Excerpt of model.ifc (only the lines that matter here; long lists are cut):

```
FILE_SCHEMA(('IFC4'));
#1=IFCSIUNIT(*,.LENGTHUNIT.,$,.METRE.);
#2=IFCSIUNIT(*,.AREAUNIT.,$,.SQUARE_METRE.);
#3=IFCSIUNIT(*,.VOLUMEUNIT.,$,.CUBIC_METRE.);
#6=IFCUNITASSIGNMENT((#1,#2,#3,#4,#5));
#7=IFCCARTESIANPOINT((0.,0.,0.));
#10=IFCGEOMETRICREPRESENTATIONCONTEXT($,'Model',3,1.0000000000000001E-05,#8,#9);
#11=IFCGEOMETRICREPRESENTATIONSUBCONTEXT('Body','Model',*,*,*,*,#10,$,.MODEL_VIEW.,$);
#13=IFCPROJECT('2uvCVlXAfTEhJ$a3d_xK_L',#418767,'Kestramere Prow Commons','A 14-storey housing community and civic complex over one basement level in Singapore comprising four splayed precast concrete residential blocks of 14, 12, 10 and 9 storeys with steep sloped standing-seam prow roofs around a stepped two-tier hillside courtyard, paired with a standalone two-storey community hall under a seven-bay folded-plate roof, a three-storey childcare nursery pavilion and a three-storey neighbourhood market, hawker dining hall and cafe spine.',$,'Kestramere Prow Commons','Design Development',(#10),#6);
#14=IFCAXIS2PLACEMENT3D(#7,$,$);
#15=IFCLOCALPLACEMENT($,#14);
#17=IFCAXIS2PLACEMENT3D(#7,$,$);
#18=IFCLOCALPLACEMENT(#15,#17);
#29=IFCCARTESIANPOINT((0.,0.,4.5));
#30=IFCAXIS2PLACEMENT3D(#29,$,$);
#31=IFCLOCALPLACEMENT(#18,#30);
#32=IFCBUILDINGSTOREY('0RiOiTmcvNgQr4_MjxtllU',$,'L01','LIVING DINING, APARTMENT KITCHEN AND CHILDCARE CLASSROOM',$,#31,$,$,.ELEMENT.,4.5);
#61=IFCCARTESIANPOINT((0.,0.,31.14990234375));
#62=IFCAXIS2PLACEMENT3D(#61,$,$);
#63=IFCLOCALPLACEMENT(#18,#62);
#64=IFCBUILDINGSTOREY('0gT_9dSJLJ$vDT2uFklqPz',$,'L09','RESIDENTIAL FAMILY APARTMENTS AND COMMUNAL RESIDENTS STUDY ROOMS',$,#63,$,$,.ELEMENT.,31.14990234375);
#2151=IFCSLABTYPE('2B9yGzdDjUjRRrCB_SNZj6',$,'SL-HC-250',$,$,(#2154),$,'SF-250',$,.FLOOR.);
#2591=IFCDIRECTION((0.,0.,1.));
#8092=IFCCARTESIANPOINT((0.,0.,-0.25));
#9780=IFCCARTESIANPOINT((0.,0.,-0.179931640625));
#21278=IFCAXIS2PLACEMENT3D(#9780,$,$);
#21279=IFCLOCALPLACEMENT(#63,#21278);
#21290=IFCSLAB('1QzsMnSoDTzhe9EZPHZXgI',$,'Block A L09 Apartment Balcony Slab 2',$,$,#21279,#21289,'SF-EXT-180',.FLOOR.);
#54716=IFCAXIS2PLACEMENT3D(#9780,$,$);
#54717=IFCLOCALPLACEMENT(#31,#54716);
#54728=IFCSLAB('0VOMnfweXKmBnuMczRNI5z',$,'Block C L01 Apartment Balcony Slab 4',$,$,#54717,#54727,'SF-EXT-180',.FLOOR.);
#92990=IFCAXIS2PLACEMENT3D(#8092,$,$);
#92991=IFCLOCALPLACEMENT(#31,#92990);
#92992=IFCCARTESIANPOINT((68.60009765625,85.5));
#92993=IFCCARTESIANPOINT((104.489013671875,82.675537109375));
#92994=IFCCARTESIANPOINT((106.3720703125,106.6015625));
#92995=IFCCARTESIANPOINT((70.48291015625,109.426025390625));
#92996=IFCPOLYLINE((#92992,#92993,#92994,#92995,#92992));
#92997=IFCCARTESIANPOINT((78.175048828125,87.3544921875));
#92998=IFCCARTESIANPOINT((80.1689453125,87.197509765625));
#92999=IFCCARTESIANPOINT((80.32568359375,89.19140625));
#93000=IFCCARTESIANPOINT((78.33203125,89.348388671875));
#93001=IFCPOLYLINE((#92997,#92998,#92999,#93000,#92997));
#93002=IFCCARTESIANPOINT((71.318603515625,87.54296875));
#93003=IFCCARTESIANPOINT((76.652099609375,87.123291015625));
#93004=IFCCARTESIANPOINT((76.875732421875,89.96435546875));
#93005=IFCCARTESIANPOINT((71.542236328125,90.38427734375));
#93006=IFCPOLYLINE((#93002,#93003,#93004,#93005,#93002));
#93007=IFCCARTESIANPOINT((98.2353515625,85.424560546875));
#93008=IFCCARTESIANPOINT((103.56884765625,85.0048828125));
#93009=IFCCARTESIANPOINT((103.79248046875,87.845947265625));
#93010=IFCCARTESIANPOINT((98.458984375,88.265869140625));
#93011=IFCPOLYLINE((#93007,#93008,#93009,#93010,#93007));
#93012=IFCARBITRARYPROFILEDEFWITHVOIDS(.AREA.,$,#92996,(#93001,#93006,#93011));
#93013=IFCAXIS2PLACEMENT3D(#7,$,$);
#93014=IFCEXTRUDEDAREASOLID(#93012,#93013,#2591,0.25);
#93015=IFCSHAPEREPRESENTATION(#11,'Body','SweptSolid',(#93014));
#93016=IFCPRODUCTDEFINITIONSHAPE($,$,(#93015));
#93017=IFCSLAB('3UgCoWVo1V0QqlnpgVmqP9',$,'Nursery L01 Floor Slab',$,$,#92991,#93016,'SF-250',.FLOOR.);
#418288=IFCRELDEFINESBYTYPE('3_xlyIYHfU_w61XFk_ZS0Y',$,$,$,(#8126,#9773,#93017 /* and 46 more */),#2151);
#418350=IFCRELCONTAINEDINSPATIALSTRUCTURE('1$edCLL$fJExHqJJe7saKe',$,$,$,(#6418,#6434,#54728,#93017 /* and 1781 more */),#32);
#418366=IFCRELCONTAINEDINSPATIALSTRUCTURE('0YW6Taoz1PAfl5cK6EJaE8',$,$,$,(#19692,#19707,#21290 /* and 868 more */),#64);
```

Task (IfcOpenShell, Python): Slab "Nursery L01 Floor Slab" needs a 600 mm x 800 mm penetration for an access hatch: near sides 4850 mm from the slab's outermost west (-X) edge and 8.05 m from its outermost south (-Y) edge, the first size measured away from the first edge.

```python
import numpy as np
import ifcopenshell
import ifcopenshell.api.feature
import ifcopenshell.api.geometry
import ifcopenshell.api.root
import ifcopenshell.geom
import ifcopenshell.util.placement
import ifcopenshell.util.representation
import ifcopenshell.util.shape
import ifcopenshell.util.unit

model = ifcopenshell.open("model.ifc")
unit_scale = ifcopenshell.util.unit.calculate_unit_scale(model)
settings = ifcopenshell.geom.settings()


def volume(element):
    """Net volume in cubic metres, openings subtracted."""
    shape = ifcopenshell.geom.create_shape(settings, element)
    return ifcopenshell.util.shape.get_volume(shape.geometry)


slab = model.by_guid("3UgCoWVo1V0QqlnpgVmqP9")
before = volume(slab)

# Extent in the slab's own axes, in metres. The edges named are its -X and -Y sides.
slab_shape = ifcopenshell.geom.create_shape(settings, slab)
vertices = ifcopenshell.util.shape.get_vertices(slab_shape.geometry)
x_min, y_min, bottom = vertices.min(axis=0)
top = vertices[:, 2].max()

opening = ifcopenshell.api.root.create_entity(model, ifc_class="IfcOpeningElement", name="Access hatch opening", predefined_type="OPENING")
context = ifcopenshell.util.representation.get_context(model, "Model", "Body", "MODEL_VIEW")
width, depth = 0.6, 0.8
outline = [(0.0, 0.0), (width, 0.0), (width, depth), (0.0, depth), (0.0, 0.0)]
# Overshoot both faces by 50 mm so the cut is clean.
shape = ifcopenshell.api.geometry.add_slab_representation(
    model, context=context, depth=top - bottom + 0.1, polyline=outline
)
ifcopenshell.api.geometry.assign_representation(model, product=opening, representation=shape)

matrix = ifcopenshell.util.placement.get_local_placement(slab.ObjectPlacement)
matrix[:, 3] = matrix @ np.append(np.array([x_min + 4.85, y_min + 8.05, bottom - 0.05]) / unit_scale, 1.0)
ifcopenshell.api.geometry.edit_object_placement(model, product=opening, matrix=matrix, is_si=False)
ifcopenshell.api.feature.add_feature(model, feature=opening, element=slab)

after = volume(slab)

print(f"slab volume {before:.3f} -> {after:.3f} m3")

model.write("model-out.ifc")
```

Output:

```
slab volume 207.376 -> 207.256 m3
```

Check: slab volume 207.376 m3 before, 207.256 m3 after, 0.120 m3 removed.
